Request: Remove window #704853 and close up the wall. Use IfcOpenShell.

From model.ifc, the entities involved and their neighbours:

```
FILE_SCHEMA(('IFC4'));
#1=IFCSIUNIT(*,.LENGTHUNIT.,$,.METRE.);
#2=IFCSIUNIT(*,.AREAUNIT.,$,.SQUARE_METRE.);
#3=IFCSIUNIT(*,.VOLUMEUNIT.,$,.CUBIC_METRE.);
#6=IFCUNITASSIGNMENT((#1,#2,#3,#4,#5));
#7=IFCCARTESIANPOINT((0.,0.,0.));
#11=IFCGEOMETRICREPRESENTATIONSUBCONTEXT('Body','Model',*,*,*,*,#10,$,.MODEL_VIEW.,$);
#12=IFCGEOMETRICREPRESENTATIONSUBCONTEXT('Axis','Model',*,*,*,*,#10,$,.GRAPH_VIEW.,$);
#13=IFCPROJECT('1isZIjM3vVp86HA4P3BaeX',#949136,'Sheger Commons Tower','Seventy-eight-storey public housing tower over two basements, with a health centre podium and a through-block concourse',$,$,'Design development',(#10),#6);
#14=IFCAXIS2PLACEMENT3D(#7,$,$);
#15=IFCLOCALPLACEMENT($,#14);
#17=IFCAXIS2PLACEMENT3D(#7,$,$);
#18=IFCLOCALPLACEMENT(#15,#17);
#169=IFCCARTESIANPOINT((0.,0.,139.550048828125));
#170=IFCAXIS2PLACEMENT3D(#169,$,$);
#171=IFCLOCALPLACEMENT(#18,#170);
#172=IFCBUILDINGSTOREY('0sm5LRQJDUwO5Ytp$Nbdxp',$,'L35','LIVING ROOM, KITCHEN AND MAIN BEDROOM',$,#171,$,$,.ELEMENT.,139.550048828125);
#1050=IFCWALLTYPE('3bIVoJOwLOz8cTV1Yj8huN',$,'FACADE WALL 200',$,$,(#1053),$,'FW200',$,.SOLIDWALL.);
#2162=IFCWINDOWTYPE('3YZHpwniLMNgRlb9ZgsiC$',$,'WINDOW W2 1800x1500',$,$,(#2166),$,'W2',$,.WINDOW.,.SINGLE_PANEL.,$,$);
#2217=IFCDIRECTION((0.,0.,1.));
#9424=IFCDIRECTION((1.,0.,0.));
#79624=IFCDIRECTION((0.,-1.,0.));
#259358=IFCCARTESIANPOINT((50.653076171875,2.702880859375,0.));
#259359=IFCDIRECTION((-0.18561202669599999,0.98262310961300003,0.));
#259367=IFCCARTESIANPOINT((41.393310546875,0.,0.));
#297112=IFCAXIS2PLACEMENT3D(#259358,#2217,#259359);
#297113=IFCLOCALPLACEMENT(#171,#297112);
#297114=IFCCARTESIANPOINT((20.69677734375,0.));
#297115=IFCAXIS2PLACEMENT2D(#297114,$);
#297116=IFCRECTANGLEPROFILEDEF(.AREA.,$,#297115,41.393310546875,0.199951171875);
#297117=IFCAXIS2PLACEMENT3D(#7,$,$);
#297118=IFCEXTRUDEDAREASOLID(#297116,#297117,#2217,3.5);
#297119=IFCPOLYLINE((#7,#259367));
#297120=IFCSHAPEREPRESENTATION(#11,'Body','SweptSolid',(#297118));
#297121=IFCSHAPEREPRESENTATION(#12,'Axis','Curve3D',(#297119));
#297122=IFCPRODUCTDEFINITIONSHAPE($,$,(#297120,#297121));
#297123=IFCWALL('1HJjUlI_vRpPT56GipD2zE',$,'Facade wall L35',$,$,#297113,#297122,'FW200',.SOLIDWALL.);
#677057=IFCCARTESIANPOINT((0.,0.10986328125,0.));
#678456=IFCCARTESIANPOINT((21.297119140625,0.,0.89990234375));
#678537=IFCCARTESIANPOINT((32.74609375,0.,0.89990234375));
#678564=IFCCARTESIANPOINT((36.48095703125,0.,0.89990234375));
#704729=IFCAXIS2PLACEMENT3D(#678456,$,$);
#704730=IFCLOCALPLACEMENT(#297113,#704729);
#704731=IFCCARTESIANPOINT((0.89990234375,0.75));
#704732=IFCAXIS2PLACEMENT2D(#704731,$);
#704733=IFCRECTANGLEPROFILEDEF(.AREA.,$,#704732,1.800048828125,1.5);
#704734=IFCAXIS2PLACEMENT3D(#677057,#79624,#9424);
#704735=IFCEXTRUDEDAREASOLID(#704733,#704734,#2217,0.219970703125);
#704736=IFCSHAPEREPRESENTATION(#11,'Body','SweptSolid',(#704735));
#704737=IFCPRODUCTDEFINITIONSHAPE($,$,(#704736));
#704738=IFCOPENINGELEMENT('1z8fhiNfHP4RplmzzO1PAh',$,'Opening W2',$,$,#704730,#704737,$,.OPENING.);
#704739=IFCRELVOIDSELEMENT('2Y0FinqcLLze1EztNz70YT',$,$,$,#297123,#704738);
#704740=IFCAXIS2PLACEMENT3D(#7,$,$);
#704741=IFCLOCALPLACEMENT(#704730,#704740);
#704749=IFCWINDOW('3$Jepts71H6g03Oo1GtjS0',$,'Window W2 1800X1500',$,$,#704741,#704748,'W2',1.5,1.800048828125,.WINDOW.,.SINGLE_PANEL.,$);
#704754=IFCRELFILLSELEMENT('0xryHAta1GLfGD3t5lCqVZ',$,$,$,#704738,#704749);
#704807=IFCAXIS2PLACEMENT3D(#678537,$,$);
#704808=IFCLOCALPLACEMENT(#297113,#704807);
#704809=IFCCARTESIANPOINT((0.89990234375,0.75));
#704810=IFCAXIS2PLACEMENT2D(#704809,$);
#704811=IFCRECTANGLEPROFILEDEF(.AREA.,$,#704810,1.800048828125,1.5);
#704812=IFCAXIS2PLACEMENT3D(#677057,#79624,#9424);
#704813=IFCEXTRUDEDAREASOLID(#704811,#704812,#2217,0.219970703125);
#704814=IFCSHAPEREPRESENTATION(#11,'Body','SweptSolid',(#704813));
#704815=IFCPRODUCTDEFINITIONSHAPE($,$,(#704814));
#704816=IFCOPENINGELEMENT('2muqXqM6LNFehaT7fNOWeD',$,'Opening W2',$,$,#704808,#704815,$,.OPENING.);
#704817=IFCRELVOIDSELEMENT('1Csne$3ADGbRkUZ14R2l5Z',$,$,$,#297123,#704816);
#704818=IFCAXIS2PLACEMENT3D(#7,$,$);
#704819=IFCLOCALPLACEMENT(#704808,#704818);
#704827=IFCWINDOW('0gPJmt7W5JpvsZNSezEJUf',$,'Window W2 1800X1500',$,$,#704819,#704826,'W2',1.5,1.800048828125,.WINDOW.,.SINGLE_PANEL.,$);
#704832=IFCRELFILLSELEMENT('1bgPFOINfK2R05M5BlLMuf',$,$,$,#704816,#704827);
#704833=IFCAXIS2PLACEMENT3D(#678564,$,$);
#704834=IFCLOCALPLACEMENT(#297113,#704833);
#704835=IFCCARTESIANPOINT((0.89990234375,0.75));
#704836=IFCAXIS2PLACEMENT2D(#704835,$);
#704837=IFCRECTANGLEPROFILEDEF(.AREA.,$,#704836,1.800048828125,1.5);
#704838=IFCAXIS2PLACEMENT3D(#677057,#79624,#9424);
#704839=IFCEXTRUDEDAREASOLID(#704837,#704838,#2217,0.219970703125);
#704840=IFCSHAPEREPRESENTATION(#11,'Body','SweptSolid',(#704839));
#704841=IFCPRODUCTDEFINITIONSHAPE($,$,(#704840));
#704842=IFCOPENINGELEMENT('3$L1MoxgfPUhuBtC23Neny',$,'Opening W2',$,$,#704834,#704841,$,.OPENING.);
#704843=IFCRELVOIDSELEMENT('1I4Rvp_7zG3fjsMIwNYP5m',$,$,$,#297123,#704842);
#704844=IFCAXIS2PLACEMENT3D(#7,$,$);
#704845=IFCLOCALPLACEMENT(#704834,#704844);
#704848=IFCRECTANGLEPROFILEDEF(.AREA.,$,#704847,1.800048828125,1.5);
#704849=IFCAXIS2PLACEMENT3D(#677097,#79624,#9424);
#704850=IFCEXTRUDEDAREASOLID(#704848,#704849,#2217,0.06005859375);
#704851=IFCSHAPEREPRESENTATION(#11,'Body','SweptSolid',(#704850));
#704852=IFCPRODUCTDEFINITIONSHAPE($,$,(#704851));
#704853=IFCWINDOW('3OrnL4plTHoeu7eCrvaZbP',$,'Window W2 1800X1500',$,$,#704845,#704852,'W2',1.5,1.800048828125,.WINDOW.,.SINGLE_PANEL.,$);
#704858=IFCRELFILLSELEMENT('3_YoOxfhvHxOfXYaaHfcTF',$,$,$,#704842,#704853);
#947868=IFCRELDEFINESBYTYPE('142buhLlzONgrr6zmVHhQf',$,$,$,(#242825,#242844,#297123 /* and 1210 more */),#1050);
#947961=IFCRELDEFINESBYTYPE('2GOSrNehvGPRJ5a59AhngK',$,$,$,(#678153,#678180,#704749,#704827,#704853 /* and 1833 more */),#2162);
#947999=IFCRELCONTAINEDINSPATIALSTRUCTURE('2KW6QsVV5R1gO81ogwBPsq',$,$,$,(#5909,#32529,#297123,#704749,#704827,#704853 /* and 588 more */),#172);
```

```python
import ifcopenshell
import ifcopenshell.api.feature
import ifcopenshell.api.root
import ifcopenshell.geom
import ifcopenshell.util.shape

model = ifcopenshell.open("model.ifc")
settings = ifcopenshell.geom.settings()


def volume(element):
    """Net volume in cubic metres, openings subtracted."""
    shape = ifcopenshell.geom.create_shape(settings, element)
    return ifcopenshell.util.shape.get_volume(shape.geometry)


window = model.by_guid("3OrnL4plTHoeu7eCrvaZbP")
opening = window.FillsVoids[0].RelatingOpeningElement
wall = opening.VoidsElements[0].RelatingBuildingElement
before = volume(wall)

ifcopenshell.api.root.remove_product(model, product=window)
ifcopenshell.api.feature.remove_feature(model, feature=opening)

after = volume(wall)

print(f"wall volume {before:.3f} -> {after:.3f} m3")

model.write("model-out.ifc")
```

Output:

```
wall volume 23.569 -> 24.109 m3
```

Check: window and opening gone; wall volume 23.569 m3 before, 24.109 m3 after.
